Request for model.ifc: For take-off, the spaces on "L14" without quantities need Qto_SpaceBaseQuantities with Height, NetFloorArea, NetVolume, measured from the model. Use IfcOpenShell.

First a look at what the model holds.

```python
import ifcopenshell
import ifcopenshell.util.element
import ifcopenshell.util.unit

model = ifcopenshell.open("model.ifc")
print(model.schema)
for unit_type in ("LENGTHUNIT", "AREAUNIT", "VOLUMEUNIT"):
    print(unit_type, ifcopenshell.util.unit.calculate_unit_scale(model, unit_type))
storey = next(s for s in model.by_type("IfcBuildingStorey") if s.Name == "L14")
spaces = [e for e in ifcopenshell.util.element.get_decomposition(storey) if e.is_a("IfcSpace")]
for e in sorted(spaces, key=lambda e: e.id()):
    print(e.id(), e.is_a(), e.Name, list(ifcopenshell.util.element.get_psets(e, qtos_only=True)), sep=" | ")
```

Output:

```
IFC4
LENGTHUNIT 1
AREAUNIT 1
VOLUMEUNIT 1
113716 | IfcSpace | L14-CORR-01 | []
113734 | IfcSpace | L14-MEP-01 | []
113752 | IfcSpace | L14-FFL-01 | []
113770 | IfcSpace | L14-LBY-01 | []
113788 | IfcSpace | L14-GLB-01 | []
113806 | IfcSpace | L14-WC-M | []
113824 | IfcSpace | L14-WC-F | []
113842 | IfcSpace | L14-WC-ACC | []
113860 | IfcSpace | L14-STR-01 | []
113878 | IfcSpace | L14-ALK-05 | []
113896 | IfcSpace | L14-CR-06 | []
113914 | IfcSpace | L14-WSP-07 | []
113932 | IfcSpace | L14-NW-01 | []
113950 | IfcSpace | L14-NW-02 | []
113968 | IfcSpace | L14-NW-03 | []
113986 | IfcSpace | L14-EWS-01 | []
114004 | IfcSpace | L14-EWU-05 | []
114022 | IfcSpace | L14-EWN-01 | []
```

```python
import ifcopenshell
import ifcopenshell.api.pset
import ifcopenshell.geom
import ifcopenshell.util.element
import ifcopenshell.util.shape
import ifcopenshell.util.unit

model = ifcopenshell.open("model.ifc")
unit_scale = ifcopenshell.util.unit.calculate_unit_scale(model)
area_scale = ifcopenshell.util.unit.calculate_unit_scale(model, "AREAUNIT")
volume_scale = ifcopenshell.util.unit.calculate_unit_scale(model, "VOLUMEUNIT")
settings = ifcopenshell.geom.settings()

storey = next(s for s in model.by_type("IfcBuildingStorey") if s.Name == "L14")
spaces = [e for e in ifcopenshell.util.element.get_decomposition(storey) if e.is_a("IfcSpace")]

for e in sorted(spaces, key=lambda e: e.id()):
    if ifcopenshell.util.element.get_psets(e, qtos_only=True, should_inherit=False):
        continue
    # Geometry comes back in metres, in the element's own axes.
    shape = ifcopenshell.geom.create_shape(settings, e)
    values = {
        "Height": ifcopenshell.util.shape.get_z(shape.geometry) / unit_scale,
        "NetFloorArea": ifcopenshell.util.shape.get_footprint_area(shape.geometry) / area_scale,
        "NetVolume": ifcopenshell.util.shape.get_volume(shape.geometry) / volume_scale,
    }
    qto = ifcopenshell.api.pset.add_qto(model, product=e, name="Qto_SpaceBaseQuantities")
    ifcopenshell.api.pset.edit_qto(model, qto=qto, properties=values)
    print(e.id(), {k: round(v, 3) for k, v in values.items()})

model.write("model_edited.ifc")
```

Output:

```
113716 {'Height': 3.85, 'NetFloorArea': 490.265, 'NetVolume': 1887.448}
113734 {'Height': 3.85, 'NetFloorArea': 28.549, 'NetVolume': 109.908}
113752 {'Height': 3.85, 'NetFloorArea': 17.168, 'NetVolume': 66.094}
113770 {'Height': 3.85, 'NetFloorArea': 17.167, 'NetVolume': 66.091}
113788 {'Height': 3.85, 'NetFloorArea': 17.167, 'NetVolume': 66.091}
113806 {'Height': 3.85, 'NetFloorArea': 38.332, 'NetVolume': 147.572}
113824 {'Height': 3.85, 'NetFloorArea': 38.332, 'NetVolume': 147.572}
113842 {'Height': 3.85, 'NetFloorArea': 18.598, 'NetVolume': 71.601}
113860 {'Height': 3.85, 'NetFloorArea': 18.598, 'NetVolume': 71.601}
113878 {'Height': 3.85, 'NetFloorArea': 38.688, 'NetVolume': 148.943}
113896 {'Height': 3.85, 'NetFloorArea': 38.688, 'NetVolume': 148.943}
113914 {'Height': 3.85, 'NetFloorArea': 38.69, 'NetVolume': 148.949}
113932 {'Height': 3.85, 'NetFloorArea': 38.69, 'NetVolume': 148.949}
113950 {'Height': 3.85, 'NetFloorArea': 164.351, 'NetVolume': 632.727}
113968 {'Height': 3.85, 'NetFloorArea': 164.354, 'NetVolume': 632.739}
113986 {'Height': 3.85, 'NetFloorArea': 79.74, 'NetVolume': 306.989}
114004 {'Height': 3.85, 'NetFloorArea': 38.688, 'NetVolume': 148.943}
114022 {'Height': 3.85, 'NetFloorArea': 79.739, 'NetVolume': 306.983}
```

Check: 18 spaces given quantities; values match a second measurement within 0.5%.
